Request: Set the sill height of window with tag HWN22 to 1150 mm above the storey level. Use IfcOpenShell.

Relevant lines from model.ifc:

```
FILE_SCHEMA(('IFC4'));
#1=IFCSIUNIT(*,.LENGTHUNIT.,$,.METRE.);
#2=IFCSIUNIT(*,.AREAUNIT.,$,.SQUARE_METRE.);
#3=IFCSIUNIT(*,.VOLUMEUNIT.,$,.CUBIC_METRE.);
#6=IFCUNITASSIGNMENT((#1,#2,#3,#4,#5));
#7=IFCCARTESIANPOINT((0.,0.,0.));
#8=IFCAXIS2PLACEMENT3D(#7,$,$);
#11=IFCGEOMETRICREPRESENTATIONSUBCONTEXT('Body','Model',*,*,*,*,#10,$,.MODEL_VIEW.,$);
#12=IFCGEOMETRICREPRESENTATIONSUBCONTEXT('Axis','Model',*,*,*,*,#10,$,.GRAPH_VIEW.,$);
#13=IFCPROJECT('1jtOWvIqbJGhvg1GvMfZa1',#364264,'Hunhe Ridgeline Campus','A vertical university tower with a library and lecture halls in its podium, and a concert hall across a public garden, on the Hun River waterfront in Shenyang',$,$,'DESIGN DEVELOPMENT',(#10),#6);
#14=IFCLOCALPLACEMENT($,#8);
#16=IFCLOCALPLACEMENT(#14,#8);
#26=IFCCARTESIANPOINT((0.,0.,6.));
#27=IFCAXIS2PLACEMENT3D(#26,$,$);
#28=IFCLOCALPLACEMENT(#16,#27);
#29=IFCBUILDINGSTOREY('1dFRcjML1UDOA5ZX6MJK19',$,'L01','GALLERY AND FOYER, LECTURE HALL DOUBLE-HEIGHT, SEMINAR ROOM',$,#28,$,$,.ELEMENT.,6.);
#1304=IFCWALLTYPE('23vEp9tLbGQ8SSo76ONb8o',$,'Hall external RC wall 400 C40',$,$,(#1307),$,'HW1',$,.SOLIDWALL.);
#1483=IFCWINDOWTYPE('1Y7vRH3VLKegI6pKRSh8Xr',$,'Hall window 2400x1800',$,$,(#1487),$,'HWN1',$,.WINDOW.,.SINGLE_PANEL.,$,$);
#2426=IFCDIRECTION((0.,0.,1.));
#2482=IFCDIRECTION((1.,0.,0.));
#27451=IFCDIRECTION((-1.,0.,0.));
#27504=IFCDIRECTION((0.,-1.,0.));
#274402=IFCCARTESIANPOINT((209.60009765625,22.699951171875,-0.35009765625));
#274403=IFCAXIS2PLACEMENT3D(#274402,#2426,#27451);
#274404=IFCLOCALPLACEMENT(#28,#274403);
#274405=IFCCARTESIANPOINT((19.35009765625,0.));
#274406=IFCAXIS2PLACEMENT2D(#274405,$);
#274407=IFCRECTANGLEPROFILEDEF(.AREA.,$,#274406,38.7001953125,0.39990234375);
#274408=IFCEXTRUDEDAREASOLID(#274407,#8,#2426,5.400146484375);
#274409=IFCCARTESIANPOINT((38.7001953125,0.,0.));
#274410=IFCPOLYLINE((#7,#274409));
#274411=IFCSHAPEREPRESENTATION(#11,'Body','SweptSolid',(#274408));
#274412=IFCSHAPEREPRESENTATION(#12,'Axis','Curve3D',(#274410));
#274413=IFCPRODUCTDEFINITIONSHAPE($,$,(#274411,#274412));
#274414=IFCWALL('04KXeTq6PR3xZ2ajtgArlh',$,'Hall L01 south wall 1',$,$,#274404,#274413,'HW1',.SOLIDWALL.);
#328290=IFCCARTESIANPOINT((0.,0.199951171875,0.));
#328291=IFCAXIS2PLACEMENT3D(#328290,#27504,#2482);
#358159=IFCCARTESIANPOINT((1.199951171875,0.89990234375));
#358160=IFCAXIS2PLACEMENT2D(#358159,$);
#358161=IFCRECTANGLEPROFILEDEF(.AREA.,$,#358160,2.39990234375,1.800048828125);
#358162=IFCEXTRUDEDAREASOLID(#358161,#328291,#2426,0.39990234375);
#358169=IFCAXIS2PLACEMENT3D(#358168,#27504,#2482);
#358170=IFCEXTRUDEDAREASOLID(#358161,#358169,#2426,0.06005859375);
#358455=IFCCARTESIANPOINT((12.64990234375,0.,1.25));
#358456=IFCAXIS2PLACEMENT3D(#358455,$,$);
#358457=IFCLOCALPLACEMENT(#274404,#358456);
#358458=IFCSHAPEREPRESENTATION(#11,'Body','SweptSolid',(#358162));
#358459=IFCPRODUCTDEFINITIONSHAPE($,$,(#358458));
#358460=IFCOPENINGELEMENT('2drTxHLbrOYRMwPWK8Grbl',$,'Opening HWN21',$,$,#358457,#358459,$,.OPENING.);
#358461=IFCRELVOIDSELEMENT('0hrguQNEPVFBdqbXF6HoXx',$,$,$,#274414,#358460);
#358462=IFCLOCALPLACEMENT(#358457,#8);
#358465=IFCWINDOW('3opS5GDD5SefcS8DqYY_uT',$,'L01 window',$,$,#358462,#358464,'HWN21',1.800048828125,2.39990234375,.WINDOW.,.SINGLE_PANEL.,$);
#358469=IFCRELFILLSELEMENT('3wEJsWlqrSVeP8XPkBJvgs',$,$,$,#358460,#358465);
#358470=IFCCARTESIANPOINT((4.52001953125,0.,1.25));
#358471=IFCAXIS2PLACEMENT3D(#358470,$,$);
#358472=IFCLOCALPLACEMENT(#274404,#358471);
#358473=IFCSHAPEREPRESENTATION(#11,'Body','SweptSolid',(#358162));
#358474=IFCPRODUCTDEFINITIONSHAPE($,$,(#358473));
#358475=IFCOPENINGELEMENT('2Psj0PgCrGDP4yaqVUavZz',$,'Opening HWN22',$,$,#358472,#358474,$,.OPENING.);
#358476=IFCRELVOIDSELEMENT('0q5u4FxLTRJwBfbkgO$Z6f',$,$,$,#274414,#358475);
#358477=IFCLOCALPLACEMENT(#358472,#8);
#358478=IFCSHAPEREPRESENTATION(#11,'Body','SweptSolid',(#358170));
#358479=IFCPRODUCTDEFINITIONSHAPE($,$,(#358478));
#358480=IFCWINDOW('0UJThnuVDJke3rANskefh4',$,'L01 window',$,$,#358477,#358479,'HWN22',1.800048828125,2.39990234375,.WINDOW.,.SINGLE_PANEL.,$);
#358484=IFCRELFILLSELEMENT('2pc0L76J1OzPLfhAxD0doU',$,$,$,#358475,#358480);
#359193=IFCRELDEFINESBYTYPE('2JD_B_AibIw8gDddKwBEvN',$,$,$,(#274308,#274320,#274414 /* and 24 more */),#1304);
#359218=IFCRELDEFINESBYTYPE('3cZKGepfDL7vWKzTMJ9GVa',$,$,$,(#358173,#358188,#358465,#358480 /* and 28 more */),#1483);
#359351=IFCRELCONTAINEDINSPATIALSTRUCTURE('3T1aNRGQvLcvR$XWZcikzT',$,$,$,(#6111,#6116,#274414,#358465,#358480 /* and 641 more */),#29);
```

```python
import numpy as np
import ifcopenshell
import ifcopenshell.api.geometry
import ifcopenshell.geom
import ifcopenshell.util.element
import ifcopenshell.util.placement
import ifcopenshell.util.shape
import ifcopenshell.util.unit

model = ifcopenshell.open("model.ifc")
unit_scale = ifcopenshell.util.unit.calculate_unit_scale(model)

window = model.by_id(358480)
opening = window.FillsVoids[0].RelatingOpeningElement
storey = ifcopenshell.util.element.get_container(window, ifc_class="IfcBuildingStorey")
level = ifcopenshell.util.placement.get_local_placement(storey.ObjectPlacement)[2, 3]

# The opening's origin need not be at the sill, so measure its lowest point.
shape = ifcopenshell.geom.create_shape(ifcopenshell.geom.settings(), opening)
bottom = ifcopenshell.util.shape.get_shape_bottom_elevation(shape, shape.geometry) / unit_scale
dz = level + 1.15 - bottom

shift = np.array([0.0, 0.0, dz])
# The window is placed relative to its opening, so it follows when the opening moves.
matrix = ifcopenshell.util.placement.get_local_placement(opening.ObjectPlacement)
matrix[:3, 3] += shift
ifcopenshell.api.geometry.edit_object_placement(
    model, product=opening, matrix=matrix, is_si=False, should_transform_children=True
)

print(f"moved by {dz * unit_scale:+.3f} m")

model.write("model_updated.ifc")
```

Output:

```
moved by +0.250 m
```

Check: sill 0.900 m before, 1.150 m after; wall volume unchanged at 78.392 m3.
